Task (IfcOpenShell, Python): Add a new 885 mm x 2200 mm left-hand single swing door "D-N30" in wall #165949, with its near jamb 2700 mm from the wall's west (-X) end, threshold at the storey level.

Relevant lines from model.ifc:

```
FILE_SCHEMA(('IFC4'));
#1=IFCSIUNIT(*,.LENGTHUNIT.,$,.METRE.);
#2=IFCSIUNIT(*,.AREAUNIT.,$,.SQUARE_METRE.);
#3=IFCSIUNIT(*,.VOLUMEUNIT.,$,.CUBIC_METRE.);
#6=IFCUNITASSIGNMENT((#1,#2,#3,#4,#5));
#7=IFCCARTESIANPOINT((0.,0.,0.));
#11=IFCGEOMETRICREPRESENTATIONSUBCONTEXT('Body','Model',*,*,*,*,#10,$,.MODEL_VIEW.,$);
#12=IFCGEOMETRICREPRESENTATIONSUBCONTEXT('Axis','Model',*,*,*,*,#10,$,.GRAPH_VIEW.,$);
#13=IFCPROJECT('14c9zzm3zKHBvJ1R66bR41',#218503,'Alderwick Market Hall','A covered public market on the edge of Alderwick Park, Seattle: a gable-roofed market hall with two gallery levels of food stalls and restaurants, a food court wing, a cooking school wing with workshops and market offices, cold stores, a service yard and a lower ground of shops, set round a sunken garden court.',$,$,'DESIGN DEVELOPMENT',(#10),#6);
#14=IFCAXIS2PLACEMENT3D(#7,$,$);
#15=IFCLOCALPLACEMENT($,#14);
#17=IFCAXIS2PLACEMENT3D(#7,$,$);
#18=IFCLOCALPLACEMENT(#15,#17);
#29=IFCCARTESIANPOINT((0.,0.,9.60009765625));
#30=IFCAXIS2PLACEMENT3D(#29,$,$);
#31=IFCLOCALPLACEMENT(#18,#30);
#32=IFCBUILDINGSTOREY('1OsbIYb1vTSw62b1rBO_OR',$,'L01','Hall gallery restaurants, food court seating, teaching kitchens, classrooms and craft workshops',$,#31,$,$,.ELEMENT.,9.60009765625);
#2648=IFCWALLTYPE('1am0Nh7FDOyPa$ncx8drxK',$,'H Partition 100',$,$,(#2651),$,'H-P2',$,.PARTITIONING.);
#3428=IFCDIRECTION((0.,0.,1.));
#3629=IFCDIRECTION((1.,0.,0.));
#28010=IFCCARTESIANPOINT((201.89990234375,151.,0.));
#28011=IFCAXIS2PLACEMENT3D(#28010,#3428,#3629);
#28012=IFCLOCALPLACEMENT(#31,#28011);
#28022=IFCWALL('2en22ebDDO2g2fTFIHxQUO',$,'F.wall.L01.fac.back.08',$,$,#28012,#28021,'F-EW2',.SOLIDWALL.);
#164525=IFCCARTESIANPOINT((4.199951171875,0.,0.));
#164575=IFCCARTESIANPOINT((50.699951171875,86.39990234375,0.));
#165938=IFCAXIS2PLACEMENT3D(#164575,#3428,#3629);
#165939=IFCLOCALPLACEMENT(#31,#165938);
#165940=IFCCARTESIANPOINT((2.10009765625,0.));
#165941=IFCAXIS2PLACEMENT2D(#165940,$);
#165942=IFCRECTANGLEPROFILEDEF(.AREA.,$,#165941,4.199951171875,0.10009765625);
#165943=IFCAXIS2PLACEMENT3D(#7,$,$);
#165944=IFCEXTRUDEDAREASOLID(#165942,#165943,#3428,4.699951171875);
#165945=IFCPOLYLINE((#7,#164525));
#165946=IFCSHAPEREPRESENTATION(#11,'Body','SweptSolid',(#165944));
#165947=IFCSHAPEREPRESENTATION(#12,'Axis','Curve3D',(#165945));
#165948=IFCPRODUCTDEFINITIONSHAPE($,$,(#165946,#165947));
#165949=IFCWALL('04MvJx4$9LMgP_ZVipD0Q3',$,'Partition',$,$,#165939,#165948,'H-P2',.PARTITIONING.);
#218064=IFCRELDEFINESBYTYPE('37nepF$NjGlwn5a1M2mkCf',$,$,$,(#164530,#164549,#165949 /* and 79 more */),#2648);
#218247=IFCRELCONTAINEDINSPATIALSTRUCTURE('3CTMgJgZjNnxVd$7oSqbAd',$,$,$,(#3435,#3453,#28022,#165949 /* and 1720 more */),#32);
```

```python
import numpy as np
import ifcopenshell
import ifcopenshell.api.feature
import ifcopenshell.api.geometry
import ifcopenshell.api.root
import ifcopenshell.api.spatial
import ifcopenshell.geom
import ifcopenshell.util.element
import ifcopenshell.util.placement
import ifcopenshell.util.representation
import ifcopenshell.util.shape
import ifcopenshell.util.unit

model = ifcopenshell.open("model.ifc")
unit_scale = ifcopenshell.util.unit.calculate_unit_scale(model)
settings = ifcopenshell.geom.settings()


def volume(element):
    """Net volume in cubic metres, openings subtracted."""
    shape = ifcopenshell.geom.create_shape(settings, element)
    return ifcopenshell.util.shape.get_volume(shape.geometry)


wall = model.by_id(165949)
storey = ifcopenshell.util.element.get_container(wall, ifc_class="IfcBuildingStorey")
context = ifcopenshell.util.representation.get_context(model, "Model", "Body", "MODEL_VIEW")
before = volume(wall)

width, height, from_end, sill = 0.885, 2.2, 2.7, 0.0  # metres

# The wall runs along its own X axis, and the end named is its -X end.
wall_shape = ifcopenshell.geom.create_shape(settings, wall)
x, y, z = ifcopenshell.util.shape.get_vertices(wall_shape.geometry).T
start = x.min() + from_end
face, thickness = float(y.min()), float(y.max() - y.min())
wall_matrix = ifcopenshell.util.placement.get_local_placement(wall.ObjectPlacement)
level = ifcopenshell.util.placement.get_local_placement(storey.ObjectPlacement)[2, 3]


def in_wall(x, y):
    """Placement at x, y metres in the wall's axes, at sill height."""
    matrix = wall_matrix.copy()
    matrix[:, 3] = wall_matrix @ np.array([x / unit_scale, y / unit_scale, 0.0, 1.0])
    matrix[2, 3] = level + sill / unit_scale
    return matrix


# Opening: a box that overshoots both wall faces by 50 mm.
opening = ifcopenshell.api.root.create_entity(model, ifc_class="IfcOpeningElement", predefined_type="OPENING")
box = ifcopenshell.api.geometry.add_wall_representation(
    model, context=context, length=width, height=height, thickness=thickness + 0.1
)
ifcopenshell.api.geometry.assign_representation(model, product=opening, representation=box)
ifcopenshell.api.geometry.edit_object_placement(model, product=opening, matrix=in_wall(start, face - 0.05), is_si=False)
ifcopenshell.api.feature.add_feature(model, feature=opening, element=wall)

door = ifcopenshell.api.root.create_entity(model, ifc_class="IfcDoor", name="D-N30", predefined_type="DOOR")
door.OverallWidth, door.OverallHeight = width / unit_scale, height / unit_scale
door.OperationType = "SINGLE_SWING_LEFT"
body = ifcopenshell.api.geometry.add_door_representation(
    model,
    context=context,
    overall_width=door.OverallWidth,
    overall_height=door.OverallHeight,
    operation_type="SINGLE_SWING_LEFT",
    lining_properties={"LiningDepth": thickness / unit_scale, "ThresholdDepth": thickness / unit_scale},
)
ifcopenshell.api.geometry.assign_representation(model, product=door, representation=body)
ifcopenshell.api.spatial.assign_container(model, products=[door], relating_structure=storey)
ifcopenshell.api.feature.add_filling(model, opening=opening, element=door)

# The lining spans the wall, so the door starts at the wall face.
ifcopenshell.api.geometry.edit_object_placement(model, product=door, matrix=in_wall(start, face), is_si=False)

after = volume(wall)

print(f"wall volume {before:.3f} -> {after:.3f} m3")

model.write("model_updated.ifc")
```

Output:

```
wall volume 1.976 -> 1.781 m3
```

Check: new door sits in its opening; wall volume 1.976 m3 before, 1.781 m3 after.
